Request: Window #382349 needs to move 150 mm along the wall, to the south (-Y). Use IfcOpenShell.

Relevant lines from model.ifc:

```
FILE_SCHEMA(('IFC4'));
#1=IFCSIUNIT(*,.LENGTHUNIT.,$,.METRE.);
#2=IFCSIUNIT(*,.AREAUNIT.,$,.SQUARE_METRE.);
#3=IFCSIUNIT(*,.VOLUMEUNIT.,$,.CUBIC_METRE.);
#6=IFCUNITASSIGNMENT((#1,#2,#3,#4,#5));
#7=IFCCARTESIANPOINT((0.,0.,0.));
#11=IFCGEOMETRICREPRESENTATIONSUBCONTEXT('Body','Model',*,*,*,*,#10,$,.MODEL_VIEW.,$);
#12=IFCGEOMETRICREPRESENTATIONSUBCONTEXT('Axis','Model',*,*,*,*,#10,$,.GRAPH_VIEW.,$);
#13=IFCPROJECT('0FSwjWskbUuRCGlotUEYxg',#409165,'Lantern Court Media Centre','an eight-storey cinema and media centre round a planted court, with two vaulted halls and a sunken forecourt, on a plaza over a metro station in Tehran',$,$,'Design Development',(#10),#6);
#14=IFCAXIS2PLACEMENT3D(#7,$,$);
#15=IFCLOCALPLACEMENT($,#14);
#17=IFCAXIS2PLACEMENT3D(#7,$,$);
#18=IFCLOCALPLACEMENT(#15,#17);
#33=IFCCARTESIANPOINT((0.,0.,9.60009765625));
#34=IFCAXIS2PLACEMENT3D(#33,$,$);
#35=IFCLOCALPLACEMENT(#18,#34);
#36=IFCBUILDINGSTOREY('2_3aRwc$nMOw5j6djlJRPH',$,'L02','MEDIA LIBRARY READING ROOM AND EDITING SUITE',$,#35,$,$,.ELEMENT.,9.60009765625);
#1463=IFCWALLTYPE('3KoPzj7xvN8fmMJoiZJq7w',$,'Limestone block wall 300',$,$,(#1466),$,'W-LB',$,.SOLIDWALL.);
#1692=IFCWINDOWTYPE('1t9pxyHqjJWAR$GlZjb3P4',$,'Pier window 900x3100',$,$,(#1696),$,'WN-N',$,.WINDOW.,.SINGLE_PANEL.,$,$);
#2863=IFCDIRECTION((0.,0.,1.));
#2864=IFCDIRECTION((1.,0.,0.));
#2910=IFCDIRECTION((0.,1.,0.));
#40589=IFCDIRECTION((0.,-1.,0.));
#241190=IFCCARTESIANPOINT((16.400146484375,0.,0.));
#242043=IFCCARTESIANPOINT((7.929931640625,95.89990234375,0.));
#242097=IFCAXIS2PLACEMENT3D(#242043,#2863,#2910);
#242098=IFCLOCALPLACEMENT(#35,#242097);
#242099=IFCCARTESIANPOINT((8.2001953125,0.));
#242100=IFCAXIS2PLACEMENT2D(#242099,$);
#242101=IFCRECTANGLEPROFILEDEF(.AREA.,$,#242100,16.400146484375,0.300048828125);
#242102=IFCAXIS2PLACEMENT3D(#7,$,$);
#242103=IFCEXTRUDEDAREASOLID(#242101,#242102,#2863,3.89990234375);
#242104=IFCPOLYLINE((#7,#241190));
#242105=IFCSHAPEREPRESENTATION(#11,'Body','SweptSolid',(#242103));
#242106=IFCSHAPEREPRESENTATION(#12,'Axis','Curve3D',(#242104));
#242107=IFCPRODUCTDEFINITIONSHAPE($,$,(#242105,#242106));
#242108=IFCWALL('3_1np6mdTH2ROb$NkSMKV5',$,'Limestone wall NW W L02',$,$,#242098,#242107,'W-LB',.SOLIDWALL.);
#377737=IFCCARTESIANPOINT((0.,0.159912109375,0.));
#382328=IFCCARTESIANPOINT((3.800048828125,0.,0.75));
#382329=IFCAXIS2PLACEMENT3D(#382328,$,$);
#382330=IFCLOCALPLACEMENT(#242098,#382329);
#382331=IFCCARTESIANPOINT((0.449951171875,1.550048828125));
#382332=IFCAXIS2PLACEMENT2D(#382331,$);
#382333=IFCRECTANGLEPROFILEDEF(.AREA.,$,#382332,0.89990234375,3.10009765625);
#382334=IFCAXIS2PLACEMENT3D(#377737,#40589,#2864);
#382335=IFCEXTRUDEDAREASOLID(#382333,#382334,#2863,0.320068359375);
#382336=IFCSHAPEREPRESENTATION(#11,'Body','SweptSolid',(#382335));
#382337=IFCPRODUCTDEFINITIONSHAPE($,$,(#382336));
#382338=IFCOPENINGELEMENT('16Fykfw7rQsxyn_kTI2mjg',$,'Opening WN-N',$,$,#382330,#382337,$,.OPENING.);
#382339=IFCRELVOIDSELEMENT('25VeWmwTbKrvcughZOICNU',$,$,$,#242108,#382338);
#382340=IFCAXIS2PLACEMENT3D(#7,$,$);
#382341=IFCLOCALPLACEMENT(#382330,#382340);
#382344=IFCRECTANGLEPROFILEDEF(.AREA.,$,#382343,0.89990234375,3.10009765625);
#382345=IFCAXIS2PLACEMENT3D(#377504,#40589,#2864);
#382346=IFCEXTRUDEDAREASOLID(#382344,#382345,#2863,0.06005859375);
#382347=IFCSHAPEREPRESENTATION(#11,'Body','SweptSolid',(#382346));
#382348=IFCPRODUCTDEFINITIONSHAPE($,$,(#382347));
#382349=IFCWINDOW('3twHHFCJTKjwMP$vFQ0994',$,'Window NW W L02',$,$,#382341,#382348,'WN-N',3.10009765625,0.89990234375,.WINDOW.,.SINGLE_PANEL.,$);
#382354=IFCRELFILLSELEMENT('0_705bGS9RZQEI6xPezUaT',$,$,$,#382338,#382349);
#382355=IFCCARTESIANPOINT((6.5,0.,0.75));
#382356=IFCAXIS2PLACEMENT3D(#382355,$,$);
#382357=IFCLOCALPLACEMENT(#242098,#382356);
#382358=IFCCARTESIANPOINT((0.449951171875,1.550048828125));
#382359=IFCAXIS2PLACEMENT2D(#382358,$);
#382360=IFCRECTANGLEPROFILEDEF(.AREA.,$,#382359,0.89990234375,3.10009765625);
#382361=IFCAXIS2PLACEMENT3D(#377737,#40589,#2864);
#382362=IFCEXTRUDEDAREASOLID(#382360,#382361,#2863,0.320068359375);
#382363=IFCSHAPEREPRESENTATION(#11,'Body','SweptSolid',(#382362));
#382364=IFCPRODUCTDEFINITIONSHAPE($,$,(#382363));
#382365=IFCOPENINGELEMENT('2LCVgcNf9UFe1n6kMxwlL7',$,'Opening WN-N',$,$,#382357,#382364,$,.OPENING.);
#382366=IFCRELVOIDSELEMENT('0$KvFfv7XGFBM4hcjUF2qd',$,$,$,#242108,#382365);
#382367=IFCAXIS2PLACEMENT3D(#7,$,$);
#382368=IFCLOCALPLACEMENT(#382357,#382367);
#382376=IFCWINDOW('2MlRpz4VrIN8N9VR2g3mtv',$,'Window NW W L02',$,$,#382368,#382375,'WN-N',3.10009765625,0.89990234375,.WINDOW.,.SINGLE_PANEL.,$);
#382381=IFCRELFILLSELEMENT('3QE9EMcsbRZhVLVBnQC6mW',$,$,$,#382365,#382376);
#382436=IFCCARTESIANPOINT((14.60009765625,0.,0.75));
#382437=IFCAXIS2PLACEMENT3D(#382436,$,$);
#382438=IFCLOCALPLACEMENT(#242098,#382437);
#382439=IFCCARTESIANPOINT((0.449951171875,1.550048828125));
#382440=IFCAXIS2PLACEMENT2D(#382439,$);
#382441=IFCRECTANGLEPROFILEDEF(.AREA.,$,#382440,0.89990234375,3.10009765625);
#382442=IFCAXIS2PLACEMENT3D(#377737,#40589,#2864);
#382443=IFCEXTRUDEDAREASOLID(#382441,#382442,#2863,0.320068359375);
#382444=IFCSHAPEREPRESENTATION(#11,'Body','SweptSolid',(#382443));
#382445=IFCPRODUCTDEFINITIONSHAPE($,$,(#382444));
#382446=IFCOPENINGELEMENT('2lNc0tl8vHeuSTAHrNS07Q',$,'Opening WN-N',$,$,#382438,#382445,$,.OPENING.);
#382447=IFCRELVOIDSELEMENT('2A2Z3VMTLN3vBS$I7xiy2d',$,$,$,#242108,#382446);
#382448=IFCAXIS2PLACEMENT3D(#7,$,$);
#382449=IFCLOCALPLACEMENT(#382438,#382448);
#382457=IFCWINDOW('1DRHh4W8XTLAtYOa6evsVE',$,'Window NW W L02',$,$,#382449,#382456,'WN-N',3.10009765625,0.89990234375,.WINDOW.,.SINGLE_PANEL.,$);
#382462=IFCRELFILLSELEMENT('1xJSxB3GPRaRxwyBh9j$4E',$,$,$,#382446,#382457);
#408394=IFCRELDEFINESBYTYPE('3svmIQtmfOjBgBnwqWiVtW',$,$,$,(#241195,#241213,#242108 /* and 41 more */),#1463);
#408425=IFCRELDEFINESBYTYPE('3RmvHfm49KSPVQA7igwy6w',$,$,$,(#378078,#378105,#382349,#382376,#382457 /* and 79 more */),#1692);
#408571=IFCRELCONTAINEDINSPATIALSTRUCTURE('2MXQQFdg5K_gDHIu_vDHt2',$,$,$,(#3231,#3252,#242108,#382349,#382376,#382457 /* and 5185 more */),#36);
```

```python
import ifcopenshell
import ifcopenshell.api.geometry
import ifcopenshell.util.placement

model = ifcopenshell.open("model.ifc")

window = model.by_id(382349)
opening = window.FillsVoids[0].RelatingOpeningElement
wall = opening.VoidsElements[0].RelatingBuildingElement

wall_matrix = ifcopenshell.util.placement.get_local_placement(wall.ObjectPlacement)
shift = wall_matrix[:3, 0] * -0.15
before = ifcopenshell.util.placement.get_local_placement(window.ObjectPlacement)[:3, 3].copy()

# The window is placed relative to its opening, so it follows when the opening moves.
matrix = ifcopenshell.util.placement.get_local_placement(opening.ObjectPlacement)
matrix[:3, 3] += shift
ifcopenshell.api.geometry.edit_object_placement(
    model, product=opening, matrix=matrix, is_si=False, should_transform_children=True
)

after = ifcopenshell.util.placement.get_local_placement(window.ObjectPlacement)[:3, 3]
print("window moved by", (after - before).round(3) + 0.0)

model.write("model_edited.ifc")
```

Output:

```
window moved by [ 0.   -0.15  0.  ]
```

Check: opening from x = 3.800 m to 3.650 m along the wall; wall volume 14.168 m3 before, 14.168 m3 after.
